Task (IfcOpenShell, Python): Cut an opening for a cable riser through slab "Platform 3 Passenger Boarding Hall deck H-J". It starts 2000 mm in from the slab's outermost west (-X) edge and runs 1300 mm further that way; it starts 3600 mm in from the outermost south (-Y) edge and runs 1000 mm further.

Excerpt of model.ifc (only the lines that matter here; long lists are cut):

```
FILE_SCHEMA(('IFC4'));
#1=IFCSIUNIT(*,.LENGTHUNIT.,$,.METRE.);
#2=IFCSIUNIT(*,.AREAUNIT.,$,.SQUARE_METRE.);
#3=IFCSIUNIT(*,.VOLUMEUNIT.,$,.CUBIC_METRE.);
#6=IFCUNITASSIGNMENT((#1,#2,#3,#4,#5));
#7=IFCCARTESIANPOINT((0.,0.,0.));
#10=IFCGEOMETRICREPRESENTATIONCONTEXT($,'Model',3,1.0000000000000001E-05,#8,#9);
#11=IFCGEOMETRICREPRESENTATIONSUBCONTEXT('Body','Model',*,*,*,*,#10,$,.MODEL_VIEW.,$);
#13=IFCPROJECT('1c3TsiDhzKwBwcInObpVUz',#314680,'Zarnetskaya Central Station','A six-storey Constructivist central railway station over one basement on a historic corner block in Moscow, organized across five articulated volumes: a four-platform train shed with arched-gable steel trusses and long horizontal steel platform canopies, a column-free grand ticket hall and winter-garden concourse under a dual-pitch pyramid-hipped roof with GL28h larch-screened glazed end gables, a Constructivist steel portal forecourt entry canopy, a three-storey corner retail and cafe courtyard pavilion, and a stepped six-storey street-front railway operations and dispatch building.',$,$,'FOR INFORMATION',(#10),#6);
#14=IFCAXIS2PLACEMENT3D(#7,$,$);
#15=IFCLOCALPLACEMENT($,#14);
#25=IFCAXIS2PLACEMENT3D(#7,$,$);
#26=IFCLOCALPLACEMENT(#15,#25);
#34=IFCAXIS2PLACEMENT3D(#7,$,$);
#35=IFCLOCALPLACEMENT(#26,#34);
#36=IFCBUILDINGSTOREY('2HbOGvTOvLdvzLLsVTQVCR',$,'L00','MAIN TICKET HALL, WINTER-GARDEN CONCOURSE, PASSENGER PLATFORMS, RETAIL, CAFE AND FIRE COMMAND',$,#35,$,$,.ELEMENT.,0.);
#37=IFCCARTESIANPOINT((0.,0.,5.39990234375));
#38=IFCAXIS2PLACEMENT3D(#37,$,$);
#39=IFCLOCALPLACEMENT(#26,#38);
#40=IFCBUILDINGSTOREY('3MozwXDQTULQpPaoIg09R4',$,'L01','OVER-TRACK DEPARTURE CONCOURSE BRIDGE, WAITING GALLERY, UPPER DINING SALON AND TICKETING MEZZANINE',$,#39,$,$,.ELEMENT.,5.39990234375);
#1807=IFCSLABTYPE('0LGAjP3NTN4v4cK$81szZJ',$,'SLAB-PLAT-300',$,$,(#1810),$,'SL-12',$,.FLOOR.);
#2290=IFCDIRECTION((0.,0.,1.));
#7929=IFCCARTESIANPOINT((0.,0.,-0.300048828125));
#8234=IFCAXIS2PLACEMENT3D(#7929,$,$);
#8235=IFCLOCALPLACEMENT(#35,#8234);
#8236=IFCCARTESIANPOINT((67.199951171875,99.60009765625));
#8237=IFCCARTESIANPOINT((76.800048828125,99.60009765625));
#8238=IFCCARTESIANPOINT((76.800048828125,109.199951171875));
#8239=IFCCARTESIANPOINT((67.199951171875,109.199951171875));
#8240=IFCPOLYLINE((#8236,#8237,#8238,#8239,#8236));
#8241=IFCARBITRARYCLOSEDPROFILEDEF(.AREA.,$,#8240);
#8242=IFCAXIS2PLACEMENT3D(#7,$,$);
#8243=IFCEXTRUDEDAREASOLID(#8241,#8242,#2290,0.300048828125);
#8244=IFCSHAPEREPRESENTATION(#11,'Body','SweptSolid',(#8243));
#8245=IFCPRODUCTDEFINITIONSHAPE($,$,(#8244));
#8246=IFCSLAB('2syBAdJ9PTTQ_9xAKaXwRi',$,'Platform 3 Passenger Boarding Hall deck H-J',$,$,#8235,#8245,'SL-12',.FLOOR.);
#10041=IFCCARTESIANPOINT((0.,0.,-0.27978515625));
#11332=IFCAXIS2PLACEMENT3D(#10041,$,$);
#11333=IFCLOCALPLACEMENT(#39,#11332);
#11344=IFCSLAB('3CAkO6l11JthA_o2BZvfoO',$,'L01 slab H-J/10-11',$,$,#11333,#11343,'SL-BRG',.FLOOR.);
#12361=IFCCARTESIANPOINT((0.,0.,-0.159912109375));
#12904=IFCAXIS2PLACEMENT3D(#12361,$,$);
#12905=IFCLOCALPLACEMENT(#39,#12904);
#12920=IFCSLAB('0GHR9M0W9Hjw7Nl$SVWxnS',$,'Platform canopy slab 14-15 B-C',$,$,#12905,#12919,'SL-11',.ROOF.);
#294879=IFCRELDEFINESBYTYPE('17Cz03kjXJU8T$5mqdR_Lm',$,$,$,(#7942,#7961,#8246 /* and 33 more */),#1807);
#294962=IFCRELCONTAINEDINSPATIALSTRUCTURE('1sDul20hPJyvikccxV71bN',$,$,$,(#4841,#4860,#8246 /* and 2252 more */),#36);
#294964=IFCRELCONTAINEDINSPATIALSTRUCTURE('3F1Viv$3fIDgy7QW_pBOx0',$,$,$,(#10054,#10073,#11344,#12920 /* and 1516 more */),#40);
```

```python
import numpy as np
import ifcopenshell
import ifcopenshell.api.feature
import ifcopenshell.api.geometry
import ifcopenshell.api.root
import ifcopenshell.geom
import ifcopenshell.util.placement
import ifcopenshell.util.representation
import ifcopenshell.util.shape
import ifcopenshell.util.unit

model = ifcopenshell.open("model.ifc")
unit_scale = ifcopenshell.util.unit.calculate_unit_scale(model)
settings = ifcopenshell.geom.settings()


def volume(element):
    """Net volume in cubic metres, openings subtracted."""
    shape = ifcopenshell.geom.create_shape(settings, element)
    return ifcopenshell.util.shape.get_volume(shape.geometry)


slab = model.by_guid("2syBAdJ9PTTQ_9xAKaXwRi")
before = volume(slab)

# Extent in the slab's own axes, in metres. The edges named are its -X and -Y sides.
slab_shape = ifcopenshell.geom.create_shape(settings, slab)
vertices = ifcopenshell.util.shape.get_vertices(slab_shape.geometry)
x_min, y_min, bottom = vertices.min(axis=0)
top = vertices[:, 2].max()

opening = ifcopenshell.api.root.create_entity(model, ifc_class="IfcOpeningElement", name="Cable riser opening", predefined_type="OPENING")
context = ifcopenshell.util.representation.get_context(model, "Model", "Body", "MODEL_VIEW")
width, depth = 1.3, 1
outline = [(0.0, 0.0), (width, 0.0), (width, depth), (0.0, depth), (0.0, 0.0)]
# Overshoot both faces by 50 mm so the cut is clean.
shape = ifcopenshell.api.geometry.add_slab_representation(
    model, context=context, depth=top - bottom + 0.1, polyline=outline
)
ifcopenshell.api.geometry.assign_representation(model, product=opening, representation=shape)

matrix = ifcopenshell.util.placement.get_local_placement(slab.ObjectPlacement)
matrix[:, 3] = matrix @ np.append(np.array([x_min + 2, y_min + 3.6, bottom - 0.05]) / unit_scale, 1.0)
ifcopenshell.api.geometry.edit_object_placement(model, product=opening, matrix=matrix, is_si=False)
ifcopenshell.api.feature.add_feature(model, feature=opening, element=slab)

after = volume(slab)

print(f"slab volume {before:.3f} -> {after:.3f} m3")

model.write("model_edited.ifc")
```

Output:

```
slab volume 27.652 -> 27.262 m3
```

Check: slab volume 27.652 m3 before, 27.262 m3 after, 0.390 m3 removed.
